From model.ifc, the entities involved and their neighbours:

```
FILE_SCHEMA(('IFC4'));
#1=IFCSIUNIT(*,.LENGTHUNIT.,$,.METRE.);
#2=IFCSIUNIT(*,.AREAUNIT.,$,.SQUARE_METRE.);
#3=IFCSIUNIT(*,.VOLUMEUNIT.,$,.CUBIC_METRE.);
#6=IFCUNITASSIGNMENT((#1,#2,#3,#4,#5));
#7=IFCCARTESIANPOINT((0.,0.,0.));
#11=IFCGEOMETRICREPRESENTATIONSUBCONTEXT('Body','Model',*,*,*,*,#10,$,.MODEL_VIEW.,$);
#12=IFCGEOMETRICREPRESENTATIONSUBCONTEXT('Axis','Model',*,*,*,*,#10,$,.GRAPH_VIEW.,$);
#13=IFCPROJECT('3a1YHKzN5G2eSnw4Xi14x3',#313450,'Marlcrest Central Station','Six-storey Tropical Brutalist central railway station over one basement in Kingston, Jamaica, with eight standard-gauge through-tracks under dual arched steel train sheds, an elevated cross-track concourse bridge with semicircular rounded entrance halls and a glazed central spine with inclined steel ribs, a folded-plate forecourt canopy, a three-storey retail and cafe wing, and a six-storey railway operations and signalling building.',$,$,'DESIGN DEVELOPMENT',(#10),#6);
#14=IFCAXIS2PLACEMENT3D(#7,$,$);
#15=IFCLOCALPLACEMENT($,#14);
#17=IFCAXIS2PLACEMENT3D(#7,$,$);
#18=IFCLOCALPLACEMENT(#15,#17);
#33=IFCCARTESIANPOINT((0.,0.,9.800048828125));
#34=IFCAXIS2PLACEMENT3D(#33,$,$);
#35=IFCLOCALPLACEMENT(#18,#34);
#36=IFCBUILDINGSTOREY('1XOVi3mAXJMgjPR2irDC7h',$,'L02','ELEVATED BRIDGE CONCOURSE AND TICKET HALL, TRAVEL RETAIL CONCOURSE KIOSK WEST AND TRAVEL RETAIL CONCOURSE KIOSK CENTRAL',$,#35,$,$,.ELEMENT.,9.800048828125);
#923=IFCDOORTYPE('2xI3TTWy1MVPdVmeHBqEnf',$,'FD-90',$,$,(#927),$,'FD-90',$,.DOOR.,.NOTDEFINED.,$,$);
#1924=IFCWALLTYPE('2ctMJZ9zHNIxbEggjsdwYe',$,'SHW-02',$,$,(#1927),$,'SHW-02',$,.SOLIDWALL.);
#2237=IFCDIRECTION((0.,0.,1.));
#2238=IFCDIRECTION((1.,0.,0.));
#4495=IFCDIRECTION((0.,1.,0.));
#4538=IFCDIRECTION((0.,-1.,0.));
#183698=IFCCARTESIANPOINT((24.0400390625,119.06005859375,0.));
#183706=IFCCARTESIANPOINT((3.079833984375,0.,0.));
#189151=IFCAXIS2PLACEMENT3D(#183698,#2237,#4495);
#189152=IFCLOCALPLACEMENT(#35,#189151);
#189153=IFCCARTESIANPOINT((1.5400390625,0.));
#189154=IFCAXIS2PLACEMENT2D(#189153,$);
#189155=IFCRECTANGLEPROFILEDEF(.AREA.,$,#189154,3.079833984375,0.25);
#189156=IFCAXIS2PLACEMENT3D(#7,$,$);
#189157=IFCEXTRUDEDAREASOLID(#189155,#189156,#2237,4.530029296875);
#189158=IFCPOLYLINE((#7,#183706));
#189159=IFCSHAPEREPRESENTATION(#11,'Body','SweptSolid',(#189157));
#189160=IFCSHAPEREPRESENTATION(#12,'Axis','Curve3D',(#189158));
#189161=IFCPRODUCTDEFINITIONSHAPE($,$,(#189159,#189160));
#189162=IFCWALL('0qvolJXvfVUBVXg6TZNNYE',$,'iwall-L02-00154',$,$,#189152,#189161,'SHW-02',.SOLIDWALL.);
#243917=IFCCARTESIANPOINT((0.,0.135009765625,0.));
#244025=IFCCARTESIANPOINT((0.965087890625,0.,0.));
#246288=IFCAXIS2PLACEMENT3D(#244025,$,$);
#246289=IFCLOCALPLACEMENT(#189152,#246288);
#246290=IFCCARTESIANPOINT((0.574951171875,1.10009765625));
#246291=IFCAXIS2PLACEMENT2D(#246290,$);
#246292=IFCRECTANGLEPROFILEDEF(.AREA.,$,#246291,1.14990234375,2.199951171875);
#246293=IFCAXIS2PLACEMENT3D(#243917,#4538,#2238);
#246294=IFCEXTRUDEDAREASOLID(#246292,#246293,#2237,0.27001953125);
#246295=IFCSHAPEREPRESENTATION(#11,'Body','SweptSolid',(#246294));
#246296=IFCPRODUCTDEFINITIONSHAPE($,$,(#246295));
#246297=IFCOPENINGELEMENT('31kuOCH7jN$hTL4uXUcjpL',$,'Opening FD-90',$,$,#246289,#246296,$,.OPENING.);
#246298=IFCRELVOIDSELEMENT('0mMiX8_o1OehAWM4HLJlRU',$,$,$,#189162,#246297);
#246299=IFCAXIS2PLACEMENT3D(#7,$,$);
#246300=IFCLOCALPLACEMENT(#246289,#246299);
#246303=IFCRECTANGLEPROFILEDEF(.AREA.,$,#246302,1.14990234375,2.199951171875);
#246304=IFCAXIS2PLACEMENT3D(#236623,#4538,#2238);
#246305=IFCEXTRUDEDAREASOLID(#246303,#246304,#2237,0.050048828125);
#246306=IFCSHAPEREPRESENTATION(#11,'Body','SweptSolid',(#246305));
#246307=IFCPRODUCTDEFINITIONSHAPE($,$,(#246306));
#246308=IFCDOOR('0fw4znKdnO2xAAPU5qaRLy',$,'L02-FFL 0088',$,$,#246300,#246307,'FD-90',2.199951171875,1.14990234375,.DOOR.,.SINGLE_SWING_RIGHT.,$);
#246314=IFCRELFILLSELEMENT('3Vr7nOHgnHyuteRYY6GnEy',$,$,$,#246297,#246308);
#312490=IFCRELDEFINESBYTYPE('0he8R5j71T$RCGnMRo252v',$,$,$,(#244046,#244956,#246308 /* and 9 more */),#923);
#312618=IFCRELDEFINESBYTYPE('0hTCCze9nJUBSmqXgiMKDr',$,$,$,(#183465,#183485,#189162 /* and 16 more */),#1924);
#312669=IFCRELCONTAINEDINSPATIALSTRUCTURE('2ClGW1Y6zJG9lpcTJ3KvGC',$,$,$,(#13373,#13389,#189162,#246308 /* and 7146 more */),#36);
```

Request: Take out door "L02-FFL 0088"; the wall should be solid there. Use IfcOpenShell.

```python
import ifcopenshell
import ifcopenshell.api.feature
import ifcopenshell.api.root
import ifcopenshell.geom
import ifcopenshell.util.shape

model = ifcopenshell.open("model.ifc")
settings = ifcopenshell.geom.settings()


def volume(element):
    """Net volume in cubic metres, openings subtracted."""
    shape = ifcopenshell.geom.create_shape(settings, element)
    return ifcopenshell.util.shape.get_volume(shape.geometry)


door = model.by_guid("0fw4znKdnO2xAAPU5qaRLy")
opening = door.FillsVoids[0].RelatingOpeningElement
wall = opening.VoidsElements[0].RelatingBuildingElement
before = volume(wall)

ifcopenshell.api.root.remove_product(model, product=door)
ifcopenshell.api.feature.remove_feature(model, feature=opening)

after = volume(wall)

print(f"wall volume {before:.3f} -> {after:.3f} m3")

model.write("model_updated.ifc")
```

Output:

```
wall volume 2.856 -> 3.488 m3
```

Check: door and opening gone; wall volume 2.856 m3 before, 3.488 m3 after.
